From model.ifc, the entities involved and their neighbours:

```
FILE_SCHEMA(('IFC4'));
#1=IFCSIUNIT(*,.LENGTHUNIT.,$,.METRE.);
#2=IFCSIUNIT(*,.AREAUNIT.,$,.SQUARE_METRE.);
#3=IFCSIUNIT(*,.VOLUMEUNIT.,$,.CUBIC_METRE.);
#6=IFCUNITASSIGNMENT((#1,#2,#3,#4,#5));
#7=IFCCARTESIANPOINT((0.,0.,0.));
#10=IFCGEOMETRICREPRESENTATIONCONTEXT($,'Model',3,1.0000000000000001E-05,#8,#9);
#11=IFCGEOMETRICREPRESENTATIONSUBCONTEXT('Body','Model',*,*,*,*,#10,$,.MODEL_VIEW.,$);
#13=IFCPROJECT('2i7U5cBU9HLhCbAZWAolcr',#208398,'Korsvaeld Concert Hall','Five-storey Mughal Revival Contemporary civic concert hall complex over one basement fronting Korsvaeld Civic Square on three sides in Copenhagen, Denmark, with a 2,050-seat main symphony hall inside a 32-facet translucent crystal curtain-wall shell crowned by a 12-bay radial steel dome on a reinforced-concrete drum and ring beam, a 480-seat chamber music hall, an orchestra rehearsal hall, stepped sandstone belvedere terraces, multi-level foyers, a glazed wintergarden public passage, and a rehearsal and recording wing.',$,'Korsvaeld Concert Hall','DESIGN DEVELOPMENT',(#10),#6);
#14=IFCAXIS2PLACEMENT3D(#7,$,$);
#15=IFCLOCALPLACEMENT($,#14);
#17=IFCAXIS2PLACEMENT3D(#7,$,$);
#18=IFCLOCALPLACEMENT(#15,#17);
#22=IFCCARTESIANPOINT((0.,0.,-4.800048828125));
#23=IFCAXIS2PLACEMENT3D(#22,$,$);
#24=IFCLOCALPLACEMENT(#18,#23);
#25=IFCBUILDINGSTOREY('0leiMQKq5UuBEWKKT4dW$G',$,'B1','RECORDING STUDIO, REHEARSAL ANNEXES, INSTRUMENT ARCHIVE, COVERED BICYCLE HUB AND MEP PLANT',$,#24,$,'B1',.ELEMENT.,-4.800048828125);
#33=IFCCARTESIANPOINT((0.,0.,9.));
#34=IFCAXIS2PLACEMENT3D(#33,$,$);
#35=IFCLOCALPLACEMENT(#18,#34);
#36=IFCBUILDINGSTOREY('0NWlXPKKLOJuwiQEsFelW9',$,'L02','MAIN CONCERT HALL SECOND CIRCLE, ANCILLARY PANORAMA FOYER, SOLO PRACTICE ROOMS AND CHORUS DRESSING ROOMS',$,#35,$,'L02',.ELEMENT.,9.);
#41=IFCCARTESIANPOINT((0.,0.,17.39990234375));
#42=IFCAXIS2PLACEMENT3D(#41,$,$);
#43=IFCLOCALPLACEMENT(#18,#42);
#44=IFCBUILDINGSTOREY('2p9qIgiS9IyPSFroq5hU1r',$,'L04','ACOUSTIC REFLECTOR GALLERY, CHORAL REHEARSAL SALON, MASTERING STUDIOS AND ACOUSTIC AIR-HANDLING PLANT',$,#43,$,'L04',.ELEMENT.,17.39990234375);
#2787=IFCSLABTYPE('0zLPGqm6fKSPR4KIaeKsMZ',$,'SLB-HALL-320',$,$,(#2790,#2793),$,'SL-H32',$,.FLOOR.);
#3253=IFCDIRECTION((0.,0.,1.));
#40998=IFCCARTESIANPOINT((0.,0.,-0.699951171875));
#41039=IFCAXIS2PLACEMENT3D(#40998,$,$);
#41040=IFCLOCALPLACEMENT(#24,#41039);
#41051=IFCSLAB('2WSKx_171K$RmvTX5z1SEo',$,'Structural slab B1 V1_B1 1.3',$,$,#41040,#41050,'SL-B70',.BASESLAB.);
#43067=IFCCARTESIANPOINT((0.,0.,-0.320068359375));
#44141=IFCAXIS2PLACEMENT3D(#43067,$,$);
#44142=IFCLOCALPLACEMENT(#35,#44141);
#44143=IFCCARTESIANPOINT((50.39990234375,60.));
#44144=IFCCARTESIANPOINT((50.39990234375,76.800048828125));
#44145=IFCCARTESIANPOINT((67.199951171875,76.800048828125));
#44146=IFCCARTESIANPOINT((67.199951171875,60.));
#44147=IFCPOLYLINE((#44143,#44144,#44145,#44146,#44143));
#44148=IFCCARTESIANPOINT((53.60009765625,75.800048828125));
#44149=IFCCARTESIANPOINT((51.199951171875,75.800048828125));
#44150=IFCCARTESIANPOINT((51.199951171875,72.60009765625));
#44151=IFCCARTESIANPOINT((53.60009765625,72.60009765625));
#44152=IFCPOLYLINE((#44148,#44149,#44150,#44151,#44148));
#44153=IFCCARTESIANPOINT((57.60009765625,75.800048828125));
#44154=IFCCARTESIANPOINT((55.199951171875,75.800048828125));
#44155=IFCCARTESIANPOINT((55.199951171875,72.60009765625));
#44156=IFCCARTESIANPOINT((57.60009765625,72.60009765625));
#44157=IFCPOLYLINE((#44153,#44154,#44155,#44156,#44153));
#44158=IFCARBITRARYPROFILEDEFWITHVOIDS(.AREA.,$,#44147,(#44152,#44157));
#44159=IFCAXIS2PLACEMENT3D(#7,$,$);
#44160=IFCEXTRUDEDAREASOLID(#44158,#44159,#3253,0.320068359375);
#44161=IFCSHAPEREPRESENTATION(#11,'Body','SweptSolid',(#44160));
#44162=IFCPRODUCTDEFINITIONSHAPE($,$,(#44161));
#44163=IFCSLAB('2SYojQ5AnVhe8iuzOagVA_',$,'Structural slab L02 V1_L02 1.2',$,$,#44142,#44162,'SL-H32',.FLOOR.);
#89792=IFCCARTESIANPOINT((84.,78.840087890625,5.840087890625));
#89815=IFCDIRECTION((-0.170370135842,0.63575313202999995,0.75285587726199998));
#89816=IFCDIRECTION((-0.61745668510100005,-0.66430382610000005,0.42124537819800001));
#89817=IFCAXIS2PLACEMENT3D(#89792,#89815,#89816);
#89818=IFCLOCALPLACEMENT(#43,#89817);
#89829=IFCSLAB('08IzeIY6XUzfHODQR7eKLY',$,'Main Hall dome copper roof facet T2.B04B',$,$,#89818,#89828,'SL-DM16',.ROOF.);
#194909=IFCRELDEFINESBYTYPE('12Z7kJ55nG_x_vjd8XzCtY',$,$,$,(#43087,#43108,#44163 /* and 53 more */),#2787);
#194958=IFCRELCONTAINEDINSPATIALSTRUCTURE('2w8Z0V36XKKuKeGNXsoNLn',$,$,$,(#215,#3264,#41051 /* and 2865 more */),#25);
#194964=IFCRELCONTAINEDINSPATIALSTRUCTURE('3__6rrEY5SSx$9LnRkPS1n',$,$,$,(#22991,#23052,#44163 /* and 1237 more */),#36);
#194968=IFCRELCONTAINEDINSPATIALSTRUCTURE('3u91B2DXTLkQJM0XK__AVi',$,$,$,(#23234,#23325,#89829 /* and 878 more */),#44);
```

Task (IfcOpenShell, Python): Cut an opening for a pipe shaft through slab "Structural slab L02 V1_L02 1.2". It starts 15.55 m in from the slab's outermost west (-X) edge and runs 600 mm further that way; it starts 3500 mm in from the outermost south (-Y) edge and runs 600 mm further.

```python
import numpy as np
import ifcopenshell
import ifcopenshell.api.feature
import ifcopenshell.api.geometry
import ifcopenshell.api.root
import ifcopenshell.geom
import ifcopenshell.util.placement
import ifcopenshell.util.representation
import ifcopenshell.util.shape
import ifcopenshell.util.unit

model = ifcopenshell.open("model.ifc")
unit_scale = ifcopenshell.util.unit.calculate_unit_scale(model)
settings = ifcopenshell.geom.settings()


def volume(element):
    """Net volume in cubic metres, openings subtracted."""
    shape = ifcopenshell.geom.create_shape(settings, element)
    return ifcopenshell.util.shape.get_volume(shape.geometry)


slab = model.by_id(44163)
before = volume(slab)

# Extent in the slab's own axes, in metres. The edges named are its -X and -Y sides.
slab_shape = ifcopenshell.geom.create_shape(settings, slab)
vertices = ifcopenshell.util.shape.get_vertices(slab_shape.geometry)
x_min, y_min, bottom = vertices.min(axis=0)
top = vertices[:, 2].max()

opening = ifcopenshell.api.root.create_entity(model, ifc_class="IfcOpeningElement", name="Pipe shaft opening", predefined_type="OPENING")
context = ifcopenshell.util.representation.get_context(model, "Model", "Body", "MODEL_VIEW")
width, depth = 0.6, 0.6
outline = [(0.0, 0.0), (width, 0.0), (width, depth), (0.0, depth), (0.0, 0.0)]
# Overshoot both faces by 50 mm so the cut is clean.
shape = ifcopenshell.api.geometry.add_slab_representation(
    model, context=context, depth=top - bottom + 0.1, polyline=outline
)
ifcopenshell.api.geometry.assign_representation(model, product=opening, representation=shape)

matrix = ifcopenshell.util.placement.get_local_placement(slab.ObjectPlacement)
matrix[:, 3] = matrix @ np.append(np.array([x_min + 15.55, y_min + 3.5, bottom - 0.05]) / unit_scale, 1.0)
ifcopenshell.api.geometry.edit_object_placement(model, product=opening, matrix=matrix, is_si=False)
ifcopenshell.api.feature.add_feature(model, feature=opening, element=slab)

after = volume(slab)

print(f"slab volume {before:.3f} -> {after:.3f} m3")

model.write("model_edited.ifc")
```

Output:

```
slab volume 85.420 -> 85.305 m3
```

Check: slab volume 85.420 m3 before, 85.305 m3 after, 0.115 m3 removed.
